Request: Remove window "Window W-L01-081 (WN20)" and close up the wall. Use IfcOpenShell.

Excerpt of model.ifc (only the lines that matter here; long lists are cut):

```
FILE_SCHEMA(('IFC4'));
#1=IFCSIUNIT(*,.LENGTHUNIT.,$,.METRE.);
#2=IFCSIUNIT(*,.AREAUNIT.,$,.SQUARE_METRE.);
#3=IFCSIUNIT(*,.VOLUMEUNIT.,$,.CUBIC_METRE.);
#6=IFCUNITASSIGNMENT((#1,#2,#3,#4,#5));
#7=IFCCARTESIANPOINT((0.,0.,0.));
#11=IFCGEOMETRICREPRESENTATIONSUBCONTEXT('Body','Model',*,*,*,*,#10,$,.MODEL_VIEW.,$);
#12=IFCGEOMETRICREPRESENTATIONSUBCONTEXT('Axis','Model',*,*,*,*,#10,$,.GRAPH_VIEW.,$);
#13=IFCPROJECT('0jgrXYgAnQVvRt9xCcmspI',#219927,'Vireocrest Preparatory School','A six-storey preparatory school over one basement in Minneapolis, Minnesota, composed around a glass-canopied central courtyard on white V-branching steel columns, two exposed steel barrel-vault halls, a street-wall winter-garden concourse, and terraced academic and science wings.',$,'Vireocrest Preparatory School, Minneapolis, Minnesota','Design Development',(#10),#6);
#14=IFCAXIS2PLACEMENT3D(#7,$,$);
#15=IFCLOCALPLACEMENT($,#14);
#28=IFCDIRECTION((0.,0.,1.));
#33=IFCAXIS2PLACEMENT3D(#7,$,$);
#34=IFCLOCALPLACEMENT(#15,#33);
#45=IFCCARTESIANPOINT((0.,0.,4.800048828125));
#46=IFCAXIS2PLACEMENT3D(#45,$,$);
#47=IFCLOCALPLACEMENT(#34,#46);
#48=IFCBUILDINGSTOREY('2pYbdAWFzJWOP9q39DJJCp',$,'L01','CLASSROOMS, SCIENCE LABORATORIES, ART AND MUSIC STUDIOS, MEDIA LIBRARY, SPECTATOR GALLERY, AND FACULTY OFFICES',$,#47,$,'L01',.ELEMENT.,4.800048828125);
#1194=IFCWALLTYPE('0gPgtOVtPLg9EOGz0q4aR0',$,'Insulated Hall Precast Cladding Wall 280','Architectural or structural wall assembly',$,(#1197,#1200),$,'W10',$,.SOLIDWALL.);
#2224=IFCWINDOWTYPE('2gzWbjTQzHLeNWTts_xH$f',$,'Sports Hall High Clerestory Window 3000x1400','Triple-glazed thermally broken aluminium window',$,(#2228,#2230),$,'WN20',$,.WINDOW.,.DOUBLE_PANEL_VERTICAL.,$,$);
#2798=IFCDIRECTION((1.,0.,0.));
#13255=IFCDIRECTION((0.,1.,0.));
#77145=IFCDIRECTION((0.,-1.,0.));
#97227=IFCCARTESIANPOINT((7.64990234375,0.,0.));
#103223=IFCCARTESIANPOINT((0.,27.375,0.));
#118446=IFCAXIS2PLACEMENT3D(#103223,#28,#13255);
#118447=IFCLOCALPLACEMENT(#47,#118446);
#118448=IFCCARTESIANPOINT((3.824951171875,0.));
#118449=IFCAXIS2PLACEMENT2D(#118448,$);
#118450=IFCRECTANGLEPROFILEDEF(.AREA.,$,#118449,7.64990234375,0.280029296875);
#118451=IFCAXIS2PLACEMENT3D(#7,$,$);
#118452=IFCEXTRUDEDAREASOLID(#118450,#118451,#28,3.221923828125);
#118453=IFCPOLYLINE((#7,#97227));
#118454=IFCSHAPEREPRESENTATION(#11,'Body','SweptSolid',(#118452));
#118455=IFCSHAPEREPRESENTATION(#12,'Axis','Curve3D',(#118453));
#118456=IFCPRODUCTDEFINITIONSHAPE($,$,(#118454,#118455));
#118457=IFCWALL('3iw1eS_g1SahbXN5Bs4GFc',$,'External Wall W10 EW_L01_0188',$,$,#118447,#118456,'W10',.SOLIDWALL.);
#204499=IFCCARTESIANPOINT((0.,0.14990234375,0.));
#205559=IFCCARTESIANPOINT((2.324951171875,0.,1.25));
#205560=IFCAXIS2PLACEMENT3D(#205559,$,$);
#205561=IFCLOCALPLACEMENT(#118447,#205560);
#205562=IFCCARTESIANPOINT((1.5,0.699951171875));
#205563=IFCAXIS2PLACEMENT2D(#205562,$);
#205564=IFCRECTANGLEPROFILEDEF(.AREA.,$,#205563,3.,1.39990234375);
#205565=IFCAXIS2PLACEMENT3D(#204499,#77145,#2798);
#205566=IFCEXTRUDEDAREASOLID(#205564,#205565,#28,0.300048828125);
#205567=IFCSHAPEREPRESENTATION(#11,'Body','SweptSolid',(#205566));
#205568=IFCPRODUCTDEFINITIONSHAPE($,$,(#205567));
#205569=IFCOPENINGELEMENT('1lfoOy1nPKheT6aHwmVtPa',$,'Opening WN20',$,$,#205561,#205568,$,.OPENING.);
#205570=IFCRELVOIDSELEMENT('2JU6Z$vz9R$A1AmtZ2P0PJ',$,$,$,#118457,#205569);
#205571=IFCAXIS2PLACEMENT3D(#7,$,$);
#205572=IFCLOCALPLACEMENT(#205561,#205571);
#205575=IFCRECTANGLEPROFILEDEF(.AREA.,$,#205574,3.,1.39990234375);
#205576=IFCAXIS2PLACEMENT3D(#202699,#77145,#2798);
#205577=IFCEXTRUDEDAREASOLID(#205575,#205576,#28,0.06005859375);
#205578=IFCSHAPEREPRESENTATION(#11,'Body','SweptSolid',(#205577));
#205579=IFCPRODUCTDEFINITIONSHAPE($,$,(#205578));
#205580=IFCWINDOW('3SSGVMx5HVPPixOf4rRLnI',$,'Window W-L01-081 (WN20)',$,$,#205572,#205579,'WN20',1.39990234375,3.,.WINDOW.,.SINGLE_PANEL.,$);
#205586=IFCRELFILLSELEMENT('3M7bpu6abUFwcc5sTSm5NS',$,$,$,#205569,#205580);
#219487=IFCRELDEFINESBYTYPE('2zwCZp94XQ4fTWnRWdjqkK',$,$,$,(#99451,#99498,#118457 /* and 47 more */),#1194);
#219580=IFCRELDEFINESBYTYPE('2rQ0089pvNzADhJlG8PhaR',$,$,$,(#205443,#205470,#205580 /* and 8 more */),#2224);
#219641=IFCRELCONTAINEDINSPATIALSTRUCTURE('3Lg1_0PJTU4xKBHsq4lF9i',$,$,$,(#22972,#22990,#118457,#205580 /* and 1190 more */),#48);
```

```python
import ifcopenshell
import ifcopenshell.api.feature
import ifcopenshell.api.root
import ifcopenshell.geom
import ifcopenshell.util.shape

model = ifcopenshell.open("model.ifc")
settings = ifcopenshell.geom.settings()


def volume(element):
    """Net volume in cubic metres, openings subtracted."""
    shape = ifcopenshell.geom.create_shape(settings, element)
    return ifcopenshell.util.shape.get_volume(shape.geometry)


window = model.by_guid("3SSGVMx5HVPPixOf4rRLnI")
opening = window.FillsVoids[0].RelatingOpeningElement
wall = opening.VoidsElements[0].RelatingBuildingElement
before = volume(wall)

ifcopenshell.api.root.remove_product(model, product=window)
ifcopenshell.api.feature.remove_feature(model, feature=opening)

after = volume(wall)

print(f"wall volume {before:.3f} -> {after:.3f} m3")

model.write("model_updated.ifc")
```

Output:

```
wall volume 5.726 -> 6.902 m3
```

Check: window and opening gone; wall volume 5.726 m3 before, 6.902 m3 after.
